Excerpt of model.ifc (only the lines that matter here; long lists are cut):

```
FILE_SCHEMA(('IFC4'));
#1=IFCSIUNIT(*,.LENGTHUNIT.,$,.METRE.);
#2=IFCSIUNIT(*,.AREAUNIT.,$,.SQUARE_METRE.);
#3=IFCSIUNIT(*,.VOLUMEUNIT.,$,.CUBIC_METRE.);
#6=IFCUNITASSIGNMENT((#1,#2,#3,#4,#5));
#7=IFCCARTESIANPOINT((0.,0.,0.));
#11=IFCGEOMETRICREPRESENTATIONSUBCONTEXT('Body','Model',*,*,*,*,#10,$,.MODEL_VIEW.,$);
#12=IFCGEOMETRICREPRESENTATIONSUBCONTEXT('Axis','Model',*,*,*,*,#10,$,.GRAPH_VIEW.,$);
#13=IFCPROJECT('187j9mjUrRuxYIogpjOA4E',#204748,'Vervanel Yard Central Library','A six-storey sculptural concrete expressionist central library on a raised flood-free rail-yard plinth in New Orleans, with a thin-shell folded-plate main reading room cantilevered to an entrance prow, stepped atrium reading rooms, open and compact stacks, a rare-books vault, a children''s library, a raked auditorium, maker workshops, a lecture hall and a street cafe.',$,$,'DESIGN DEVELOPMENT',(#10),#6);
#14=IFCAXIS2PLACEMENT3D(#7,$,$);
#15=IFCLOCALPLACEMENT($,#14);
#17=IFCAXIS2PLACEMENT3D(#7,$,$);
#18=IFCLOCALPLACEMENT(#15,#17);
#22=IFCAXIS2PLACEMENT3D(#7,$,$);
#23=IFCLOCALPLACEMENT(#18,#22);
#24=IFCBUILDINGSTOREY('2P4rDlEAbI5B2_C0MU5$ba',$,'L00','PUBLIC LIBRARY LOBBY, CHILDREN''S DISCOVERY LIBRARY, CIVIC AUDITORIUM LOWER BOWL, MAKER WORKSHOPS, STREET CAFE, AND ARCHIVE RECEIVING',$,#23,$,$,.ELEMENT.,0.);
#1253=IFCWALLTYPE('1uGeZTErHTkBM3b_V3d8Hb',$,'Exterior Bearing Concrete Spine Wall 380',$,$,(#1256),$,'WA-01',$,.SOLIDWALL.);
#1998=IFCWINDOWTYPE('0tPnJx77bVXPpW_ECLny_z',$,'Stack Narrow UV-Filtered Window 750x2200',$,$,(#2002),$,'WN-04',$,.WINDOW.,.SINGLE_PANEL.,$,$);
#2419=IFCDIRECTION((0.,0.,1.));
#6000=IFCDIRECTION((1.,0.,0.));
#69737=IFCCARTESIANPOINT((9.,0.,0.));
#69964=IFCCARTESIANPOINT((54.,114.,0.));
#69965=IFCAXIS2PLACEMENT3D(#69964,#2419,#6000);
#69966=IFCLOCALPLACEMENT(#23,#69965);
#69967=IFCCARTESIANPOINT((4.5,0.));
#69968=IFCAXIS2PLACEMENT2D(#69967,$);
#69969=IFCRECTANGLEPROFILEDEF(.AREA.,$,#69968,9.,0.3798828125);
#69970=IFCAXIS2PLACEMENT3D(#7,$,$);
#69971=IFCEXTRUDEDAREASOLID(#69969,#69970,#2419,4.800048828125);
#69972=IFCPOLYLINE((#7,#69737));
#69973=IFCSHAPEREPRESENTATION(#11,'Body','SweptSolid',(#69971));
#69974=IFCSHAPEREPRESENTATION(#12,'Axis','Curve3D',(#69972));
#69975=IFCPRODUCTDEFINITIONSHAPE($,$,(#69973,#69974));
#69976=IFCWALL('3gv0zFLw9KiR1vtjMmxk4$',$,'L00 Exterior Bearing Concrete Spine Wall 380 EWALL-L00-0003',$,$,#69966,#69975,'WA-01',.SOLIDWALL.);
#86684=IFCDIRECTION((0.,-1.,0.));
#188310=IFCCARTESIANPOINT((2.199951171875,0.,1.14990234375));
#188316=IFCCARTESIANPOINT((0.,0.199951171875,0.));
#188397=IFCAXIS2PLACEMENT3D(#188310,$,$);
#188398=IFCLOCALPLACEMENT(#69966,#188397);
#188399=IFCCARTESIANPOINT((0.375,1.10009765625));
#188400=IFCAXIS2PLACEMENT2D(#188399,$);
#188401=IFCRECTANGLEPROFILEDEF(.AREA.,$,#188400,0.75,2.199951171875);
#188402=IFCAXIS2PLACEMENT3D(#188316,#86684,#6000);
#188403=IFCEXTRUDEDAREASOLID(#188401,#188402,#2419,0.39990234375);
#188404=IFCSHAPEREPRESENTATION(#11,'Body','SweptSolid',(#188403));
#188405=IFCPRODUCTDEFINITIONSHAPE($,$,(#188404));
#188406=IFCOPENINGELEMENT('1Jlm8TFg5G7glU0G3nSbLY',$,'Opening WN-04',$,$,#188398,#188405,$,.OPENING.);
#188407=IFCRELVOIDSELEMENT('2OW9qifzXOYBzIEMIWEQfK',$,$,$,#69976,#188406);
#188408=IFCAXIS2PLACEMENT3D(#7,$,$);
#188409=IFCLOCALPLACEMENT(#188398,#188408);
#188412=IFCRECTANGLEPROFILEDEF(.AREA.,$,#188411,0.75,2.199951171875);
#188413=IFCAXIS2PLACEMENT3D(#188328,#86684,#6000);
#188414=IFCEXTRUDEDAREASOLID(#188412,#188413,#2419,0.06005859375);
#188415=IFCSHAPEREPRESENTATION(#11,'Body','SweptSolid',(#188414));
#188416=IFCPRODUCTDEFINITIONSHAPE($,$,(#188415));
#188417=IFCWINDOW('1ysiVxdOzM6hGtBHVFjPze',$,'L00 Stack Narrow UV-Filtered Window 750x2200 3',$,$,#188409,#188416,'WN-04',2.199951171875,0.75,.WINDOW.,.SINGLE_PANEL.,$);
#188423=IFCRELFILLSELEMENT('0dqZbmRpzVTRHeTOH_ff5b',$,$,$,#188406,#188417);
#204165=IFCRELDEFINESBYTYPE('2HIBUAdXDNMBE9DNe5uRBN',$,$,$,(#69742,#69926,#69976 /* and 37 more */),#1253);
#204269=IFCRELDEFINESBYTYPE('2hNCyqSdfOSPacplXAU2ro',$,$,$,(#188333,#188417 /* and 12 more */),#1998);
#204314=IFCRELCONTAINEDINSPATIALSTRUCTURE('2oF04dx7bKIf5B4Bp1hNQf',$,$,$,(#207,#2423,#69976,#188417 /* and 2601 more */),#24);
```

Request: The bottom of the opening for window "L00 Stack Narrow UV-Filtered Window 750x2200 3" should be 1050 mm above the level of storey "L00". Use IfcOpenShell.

```python
import numpy as np
import ifcopenshell
import ifcopenshell.api.geometry
import ifcopenshell.geom
import ifcopenshell.util.element
import ifcopenshell.util.placement
import ifcopenshell.util.shape
import ifcopenshell.util.unit

model = ifcopenshell.open("model.ifc")
unit_scale = ifcopenshell.util.unit.calculate_unit_scale(model)

window = model.by_guid("1ysiVxdOzM6hGtBHVFjPze")
opening = window.FillsVoids[0].RelatingOpeningElement
storey = ifcopenshell.util.element.get_container(window, ifc_class="IfcBuildingStorey")
level = ifcopenshell.util.placement.get_local_placement(storey.ObjectPlacement)[2, 3]

# The opening's origin need not be at the sill, so measure its lowest point.
shape = ifcopenshell.geom.create_shape(ifcopenshell.geom.settings(), opening)
bottom = ifcopenshell.util.shape.get_shape_bottom_elevation(shape, shape.geometry) / unit_scale
dz = level + 1.05 / unit_scale - bottom

shift = np.array([0.0, 0.0, dz])
# The window is placed relative to its opening, so it follows when the opening moves.
matrix = ifcopenshell.util.placement.get_local_placement(opening.ObjectPlacement)
matrix[:3, 3] += shift
ifcopenshell.api.geometry.edit_object_placement(
    model, product=opening, matrix=matrix, is_si=False, should_transform_children=True
)

print(f"moved by {dz * unit_scale:+.3f} m")

model.write("model-out.ifc")
```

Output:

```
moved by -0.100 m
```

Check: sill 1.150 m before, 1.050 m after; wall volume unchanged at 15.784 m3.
